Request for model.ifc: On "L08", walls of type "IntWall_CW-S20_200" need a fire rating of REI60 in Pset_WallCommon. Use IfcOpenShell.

First a look at what the model holds.

```python
import ifcopenshell
import ifcopenshell.util.element

model = ifcopenshell.open("model.ifc")
print(model.schema)
storey = next(s for s in model.by_type("IfcBuildingStorey") if s.Name == "L08")
walls = [e for e in ifcopenshell.util.element.get_decomposition(storey) if e.is_a("IfcWall")]
seen = {}
for e in walls:
    element_type = ifcopenshell.util.element.get_type(e)
    key = (element_type.Name if element_type != e and element_type else None, ifcopenshell.util.element.get_pset(e, "Pset_WallCommon", "FireRating"))
    seen[key] = seen.get(key, 0) + 1
for (name, value), count in sorted(seen.items(), key=str):
    print(count, "x", name, "|", value)
```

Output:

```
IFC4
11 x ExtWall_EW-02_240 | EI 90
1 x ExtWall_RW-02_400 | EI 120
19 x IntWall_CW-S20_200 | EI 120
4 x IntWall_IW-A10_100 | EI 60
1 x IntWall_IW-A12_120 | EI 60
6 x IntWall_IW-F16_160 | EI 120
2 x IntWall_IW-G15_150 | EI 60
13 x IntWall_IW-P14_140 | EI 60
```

```python
import ifcopenshell
import ifcopenshell.api.pset
import ifcopenshell.util.element

model = ifcopenshell.open("model.ifc")

storey = next(s for s in model.by_type("IfcBuildingStorey") if s.Name == "L08")
walls = [e for e in ifcopenshell.util.element.get_decomposition(storey) if e.is_a("IfcWall")]

count = 0
for e in walls:
    element_type = ifcopenshell.util.element.get_type(e)
    if element_type in (None, e) or element_type.Name != "IntWall_CW-S20_200":
        continue
    # add_pset returns the element's existing set when there is one.
    pset = ifcopenshell.api.pset.add_pset(model, product=e, name="Pset_WallCommon")
    ifcopenshell.api.pset.edit_pset(model, pset=pset, properties={"FireRating": "REI60"})
    count += 1

print(count, "walls updated")

model.write("model_v2.ifc")
```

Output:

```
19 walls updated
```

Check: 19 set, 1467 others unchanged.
